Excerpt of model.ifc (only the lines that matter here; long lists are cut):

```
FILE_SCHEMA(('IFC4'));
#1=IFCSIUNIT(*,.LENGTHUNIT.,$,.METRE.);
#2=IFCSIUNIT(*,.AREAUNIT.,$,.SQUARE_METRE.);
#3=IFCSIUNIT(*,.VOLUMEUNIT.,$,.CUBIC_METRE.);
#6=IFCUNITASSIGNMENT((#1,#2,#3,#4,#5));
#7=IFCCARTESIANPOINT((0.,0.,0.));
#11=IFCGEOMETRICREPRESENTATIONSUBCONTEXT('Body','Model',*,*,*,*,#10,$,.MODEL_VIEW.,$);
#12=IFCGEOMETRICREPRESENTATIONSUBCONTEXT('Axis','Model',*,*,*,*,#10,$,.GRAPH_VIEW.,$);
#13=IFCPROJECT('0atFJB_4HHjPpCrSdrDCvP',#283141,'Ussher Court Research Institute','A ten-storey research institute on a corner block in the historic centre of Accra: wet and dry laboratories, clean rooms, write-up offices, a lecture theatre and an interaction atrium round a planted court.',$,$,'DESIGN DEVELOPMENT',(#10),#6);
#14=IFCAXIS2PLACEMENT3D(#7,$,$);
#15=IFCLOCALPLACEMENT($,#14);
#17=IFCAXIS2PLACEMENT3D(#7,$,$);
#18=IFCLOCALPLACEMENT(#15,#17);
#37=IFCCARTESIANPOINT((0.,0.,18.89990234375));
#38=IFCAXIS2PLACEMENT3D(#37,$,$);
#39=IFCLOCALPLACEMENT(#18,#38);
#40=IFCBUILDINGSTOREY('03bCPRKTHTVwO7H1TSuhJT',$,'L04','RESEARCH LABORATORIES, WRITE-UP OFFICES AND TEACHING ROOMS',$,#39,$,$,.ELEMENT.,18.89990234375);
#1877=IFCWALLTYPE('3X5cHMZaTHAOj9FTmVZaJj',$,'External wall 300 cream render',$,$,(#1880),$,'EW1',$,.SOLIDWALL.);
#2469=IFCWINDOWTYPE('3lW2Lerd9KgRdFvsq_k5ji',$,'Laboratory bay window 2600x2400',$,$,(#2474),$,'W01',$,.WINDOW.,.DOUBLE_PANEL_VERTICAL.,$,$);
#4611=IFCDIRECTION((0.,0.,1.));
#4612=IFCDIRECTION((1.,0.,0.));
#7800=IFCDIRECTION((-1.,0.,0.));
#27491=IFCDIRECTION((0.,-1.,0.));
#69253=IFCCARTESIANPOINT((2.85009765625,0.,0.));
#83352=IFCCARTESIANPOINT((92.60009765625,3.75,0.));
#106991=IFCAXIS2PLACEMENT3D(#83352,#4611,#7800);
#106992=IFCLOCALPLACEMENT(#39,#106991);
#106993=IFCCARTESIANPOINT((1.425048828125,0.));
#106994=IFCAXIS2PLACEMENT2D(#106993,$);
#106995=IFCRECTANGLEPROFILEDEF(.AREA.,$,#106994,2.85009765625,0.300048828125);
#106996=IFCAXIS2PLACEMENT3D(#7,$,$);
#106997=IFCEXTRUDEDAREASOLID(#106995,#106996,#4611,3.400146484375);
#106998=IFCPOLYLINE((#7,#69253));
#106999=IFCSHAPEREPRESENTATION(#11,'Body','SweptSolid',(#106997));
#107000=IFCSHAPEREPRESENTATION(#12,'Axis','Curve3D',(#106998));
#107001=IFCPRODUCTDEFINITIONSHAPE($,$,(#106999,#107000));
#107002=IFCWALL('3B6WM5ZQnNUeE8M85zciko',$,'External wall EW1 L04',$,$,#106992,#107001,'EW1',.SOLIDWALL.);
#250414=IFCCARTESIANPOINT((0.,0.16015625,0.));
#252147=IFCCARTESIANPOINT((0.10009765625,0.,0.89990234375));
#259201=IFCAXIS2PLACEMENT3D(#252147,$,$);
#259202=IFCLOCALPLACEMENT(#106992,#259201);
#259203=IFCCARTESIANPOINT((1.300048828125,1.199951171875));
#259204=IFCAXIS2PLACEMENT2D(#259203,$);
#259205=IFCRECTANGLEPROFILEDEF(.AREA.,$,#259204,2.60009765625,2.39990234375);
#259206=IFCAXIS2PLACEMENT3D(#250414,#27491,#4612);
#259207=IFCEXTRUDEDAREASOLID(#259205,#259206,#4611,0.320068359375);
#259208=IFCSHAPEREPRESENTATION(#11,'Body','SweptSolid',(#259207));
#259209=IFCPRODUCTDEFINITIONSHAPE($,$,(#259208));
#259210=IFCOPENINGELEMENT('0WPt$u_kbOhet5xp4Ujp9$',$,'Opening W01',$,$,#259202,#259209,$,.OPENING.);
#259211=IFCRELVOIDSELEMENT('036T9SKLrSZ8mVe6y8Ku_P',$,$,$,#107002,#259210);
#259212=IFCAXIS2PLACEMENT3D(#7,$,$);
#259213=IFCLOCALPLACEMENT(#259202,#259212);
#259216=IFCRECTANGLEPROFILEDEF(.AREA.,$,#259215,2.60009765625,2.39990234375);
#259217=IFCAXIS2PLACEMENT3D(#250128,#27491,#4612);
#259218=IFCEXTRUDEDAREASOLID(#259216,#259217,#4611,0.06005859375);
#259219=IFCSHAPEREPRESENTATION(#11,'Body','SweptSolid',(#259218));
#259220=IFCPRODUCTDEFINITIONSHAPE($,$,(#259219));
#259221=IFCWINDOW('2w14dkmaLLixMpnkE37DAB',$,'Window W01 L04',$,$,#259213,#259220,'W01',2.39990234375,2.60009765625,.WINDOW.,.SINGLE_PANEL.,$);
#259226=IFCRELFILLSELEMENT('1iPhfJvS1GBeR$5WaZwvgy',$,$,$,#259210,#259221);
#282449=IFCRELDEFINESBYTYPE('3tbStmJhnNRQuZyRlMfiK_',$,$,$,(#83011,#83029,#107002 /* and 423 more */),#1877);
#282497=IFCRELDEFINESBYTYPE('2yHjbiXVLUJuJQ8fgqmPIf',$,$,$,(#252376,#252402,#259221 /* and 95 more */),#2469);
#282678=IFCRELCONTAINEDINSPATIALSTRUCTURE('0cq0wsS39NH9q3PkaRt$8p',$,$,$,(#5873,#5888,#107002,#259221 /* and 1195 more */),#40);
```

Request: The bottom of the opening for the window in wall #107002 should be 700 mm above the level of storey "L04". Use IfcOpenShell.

```python
import numpy as np
import ifcopenshell
import ifcopenshell.api.geometry
import ifcopenshell.geom
import ifcopenshell.util.element
import ifcopenshell.util.placement
import ifcopenshell.util.shape
import ifcopenshell.util.unit

model = ifcopenshell.open("model.ifc")
unit_scale = ifcopenshell.util.unit.calculate_unit_scale(model)

window = model.by_guid("2w14dkmaLLixMpnkE37DAB")
opening = window.FillsVoids[0].RelatingOpeningElement
storey = ifcopenshell.util.element.get_container(window, ifc_class="IfcBuildingStorey")
level = ifcopenshell.util.placement.get_local_placement(storey.ObjectPlacement)[2, 3]

# The opening's origin need not be at the sill, so measure its lowest point.
shape = ifcopenshell.geom.create_shape(ifcopenshell.geom.settings(), opening)
bottom = ifcopenshell.util.shape.get_shape_bottom_elevation(shape, shape.geometry) / unit_scale
dz = level + 0.7 / unit_scale - bottom

shift = np.array([0.0, 0.0, dz])
# The window is placed relative to its opening, so it follows when the opening moves.
matrix = ifcopenshell.util.placement.get_local_placement(opening.ObjectPlacement)
matrix[:3, 3] += shift
ifcopenshell.api.geometry.edit_object_placement(
    model, product=opening, matrix=matrix, is_si=False, should_transform_children=True
)

print(f"moved by {dz * unit_scale:+.3f} m")

model.write("model_updated.ifc")
```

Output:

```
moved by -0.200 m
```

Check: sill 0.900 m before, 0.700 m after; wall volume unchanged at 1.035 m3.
